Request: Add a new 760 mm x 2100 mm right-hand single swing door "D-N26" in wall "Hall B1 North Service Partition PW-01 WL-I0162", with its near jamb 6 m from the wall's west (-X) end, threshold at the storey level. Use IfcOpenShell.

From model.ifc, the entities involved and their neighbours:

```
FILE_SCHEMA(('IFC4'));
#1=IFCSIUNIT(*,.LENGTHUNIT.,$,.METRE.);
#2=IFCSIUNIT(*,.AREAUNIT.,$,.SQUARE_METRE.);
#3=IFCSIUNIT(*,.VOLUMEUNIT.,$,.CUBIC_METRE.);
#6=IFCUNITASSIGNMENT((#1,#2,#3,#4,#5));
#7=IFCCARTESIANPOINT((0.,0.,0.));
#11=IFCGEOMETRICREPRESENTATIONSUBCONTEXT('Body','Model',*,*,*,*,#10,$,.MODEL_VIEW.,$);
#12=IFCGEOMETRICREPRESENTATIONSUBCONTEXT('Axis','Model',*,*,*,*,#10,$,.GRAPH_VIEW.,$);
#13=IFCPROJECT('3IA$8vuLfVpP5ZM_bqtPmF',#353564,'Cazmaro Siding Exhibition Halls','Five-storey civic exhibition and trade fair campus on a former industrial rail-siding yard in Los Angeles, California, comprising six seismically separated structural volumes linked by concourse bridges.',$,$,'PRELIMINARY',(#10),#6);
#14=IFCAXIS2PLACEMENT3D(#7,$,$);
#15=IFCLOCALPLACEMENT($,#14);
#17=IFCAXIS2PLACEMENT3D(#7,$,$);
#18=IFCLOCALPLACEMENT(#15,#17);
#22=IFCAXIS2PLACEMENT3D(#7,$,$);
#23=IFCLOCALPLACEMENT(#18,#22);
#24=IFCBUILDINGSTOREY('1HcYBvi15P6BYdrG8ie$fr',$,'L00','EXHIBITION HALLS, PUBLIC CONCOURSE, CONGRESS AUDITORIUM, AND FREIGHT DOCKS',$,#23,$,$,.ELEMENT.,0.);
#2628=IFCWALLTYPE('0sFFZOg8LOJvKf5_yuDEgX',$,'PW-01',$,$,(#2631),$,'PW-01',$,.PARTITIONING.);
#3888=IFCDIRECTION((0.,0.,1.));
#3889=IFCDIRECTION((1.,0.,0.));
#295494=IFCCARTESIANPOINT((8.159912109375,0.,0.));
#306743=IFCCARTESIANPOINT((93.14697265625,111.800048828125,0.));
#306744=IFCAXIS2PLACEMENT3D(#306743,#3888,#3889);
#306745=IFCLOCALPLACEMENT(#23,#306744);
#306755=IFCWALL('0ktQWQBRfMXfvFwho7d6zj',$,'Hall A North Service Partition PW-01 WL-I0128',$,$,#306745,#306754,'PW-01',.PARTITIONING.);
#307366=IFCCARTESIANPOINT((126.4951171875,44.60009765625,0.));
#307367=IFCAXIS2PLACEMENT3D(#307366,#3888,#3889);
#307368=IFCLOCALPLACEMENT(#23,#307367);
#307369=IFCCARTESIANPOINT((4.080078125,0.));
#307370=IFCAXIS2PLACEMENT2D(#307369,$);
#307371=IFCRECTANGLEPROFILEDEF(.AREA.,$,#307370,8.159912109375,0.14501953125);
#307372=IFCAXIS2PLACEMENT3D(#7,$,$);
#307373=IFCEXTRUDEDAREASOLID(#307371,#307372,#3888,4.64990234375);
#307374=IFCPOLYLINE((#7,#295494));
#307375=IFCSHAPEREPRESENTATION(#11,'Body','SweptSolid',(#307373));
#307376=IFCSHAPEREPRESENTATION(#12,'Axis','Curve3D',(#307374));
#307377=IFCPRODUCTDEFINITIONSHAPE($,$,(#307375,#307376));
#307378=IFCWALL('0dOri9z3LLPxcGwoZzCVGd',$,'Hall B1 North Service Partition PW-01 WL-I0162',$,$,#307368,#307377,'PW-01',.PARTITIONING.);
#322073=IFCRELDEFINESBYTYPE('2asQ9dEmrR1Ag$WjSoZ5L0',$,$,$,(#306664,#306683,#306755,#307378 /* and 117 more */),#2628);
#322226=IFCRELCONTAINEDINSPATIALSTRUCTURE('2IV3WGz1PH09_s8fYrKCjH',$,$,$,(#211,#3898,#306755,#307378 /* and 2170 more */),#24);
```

```python
import numpy as np
import ifcopenshell
import ifcopenshell.api.feature
import ifcopenshell.api.geometry
import ifcopenshell.api.root
import ifcopenshell.api.spatial
import ifcopenshell.geom
import ifcopenshell.util.element
import ifcopenshell.util.placement
import ifcopenshell.util.representation
import ifcopenshell.util.shape
import ifcopenshell.util.unit

model = ifcopenshell.open("model.ifc")
unit_scale = ifcopenshell.util.unit.calculate_unit_scale(model)
settings = ifcopenshell.geom.settings()


def volume(element):
    """Net volume in cubic metres, openings subtracted."""
    shape = ifcopenshell.geom.create_shape(settings, element)
    return ifcopenshell.util.shape.get_volume(shape.geometry)


wall = model.by_id(307378)
storey = ifcopenshell.util.element.get_container(wall, ifc_class="IfcBuildingStorey")
context = ifcopenshell.util.representation.get_context(model, "Model", "Body", "MODEL_VIEW")
before = volume(wall)

width, height, from_end, sill = 0.76, 2.1, 6, 0.0  # metres

# The wall runs along its own X axis, and the end named is its -X end.
wall_shape = ifcopenshell.geom.create_shape(settings, wall)
x, y, z = ifcopenshell.util.shape.get_vertices(wall_shape.geometry).T
start = x.min() + from_end
face, thickness = float(y.min()), float(y.max() - y.min())
wall_matrix = ifcopenshell.util.placement.get_local_placement(wall.ObjectPlacement)
level = ifcopenshell.util.placement.get_local_placement(storey.ObjectPlacement)[2, 3]


def in_wall(x, y):
    """Placement at x, y metres in the wall's axes, at sill height."""
    matrix = wall_matrix.copy()
    matrix[:, 3] = wall_matrix @ np.array([x / unit_scale, y / unit_scale, 0.0, 1.0])
    matrix[2, 3] = level + sill / unit_scale
    return matrix


# Opening: a box that overshoots both wall faces by 50 mm.
opening = ifcopenshell.api.root.create_entity(model, ifc_class="IfcOpeningElement", predefined_type="OPENING")
box = ifcopenshell.api.geometry.add_wall_representation(
    model, context=context, length=width, height=height, thickness=thickness + 0.1
)
ifcopenshell.api.geometry.assign_representation(model, product=opening, representation=box)
ifcopenshell.api.geometry.edit_object_placement(model, product=opening, matrix=in_wall(start, face - 0.05), is_si=False)
ifcopenshell.api.feature.add_feature(model, feature=opening, element=wall)

door = ifcopenshell.api.root.create_entity(model, ifc_class="IfcDoor", name="D-N26", predefined_type="DOOR")
door.OverallWidth, door.OverallHeight = width / unit_scale, height / unit_scale
door.OperationType = "SINGLE_SWING_RIGHT"
body = ifcopenshell.api.geometry.add_door_representation(
    model,
    context=context,
    overall_width=door.OverallWidth,
    overall_height=door.OverallHeight,
    operation_type="SINGLE_SWING_RIGHT",
    lining_properties={"LiningDepth": thickness / unit_scale, "ThresholdDepth": thickness / unit_scale},
)
ifcopenshell.api.geometry.assign_representation(model, product=door, representation=body)
ifcopenshell.api.spatial.assign_container(model, products=[door], relating_structure=storey)
ifcopenshell.api.feature.add_filling(model, opening=opening, element=door)

# The lining spans the wall, so the door starts at the wall face.
ifcopenshell.api.geometry.edit_object_placement(model, product=door, matrix=in_wall(start, face), is_si=False)

after = volume(wall)

print(f"wall volume {before:.3f} -> {after:.3f} m3")

model.write("model_edited.ifc")
```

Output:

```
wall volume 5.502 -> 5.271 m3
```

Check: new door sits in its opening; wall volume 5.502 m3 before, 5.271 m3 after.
